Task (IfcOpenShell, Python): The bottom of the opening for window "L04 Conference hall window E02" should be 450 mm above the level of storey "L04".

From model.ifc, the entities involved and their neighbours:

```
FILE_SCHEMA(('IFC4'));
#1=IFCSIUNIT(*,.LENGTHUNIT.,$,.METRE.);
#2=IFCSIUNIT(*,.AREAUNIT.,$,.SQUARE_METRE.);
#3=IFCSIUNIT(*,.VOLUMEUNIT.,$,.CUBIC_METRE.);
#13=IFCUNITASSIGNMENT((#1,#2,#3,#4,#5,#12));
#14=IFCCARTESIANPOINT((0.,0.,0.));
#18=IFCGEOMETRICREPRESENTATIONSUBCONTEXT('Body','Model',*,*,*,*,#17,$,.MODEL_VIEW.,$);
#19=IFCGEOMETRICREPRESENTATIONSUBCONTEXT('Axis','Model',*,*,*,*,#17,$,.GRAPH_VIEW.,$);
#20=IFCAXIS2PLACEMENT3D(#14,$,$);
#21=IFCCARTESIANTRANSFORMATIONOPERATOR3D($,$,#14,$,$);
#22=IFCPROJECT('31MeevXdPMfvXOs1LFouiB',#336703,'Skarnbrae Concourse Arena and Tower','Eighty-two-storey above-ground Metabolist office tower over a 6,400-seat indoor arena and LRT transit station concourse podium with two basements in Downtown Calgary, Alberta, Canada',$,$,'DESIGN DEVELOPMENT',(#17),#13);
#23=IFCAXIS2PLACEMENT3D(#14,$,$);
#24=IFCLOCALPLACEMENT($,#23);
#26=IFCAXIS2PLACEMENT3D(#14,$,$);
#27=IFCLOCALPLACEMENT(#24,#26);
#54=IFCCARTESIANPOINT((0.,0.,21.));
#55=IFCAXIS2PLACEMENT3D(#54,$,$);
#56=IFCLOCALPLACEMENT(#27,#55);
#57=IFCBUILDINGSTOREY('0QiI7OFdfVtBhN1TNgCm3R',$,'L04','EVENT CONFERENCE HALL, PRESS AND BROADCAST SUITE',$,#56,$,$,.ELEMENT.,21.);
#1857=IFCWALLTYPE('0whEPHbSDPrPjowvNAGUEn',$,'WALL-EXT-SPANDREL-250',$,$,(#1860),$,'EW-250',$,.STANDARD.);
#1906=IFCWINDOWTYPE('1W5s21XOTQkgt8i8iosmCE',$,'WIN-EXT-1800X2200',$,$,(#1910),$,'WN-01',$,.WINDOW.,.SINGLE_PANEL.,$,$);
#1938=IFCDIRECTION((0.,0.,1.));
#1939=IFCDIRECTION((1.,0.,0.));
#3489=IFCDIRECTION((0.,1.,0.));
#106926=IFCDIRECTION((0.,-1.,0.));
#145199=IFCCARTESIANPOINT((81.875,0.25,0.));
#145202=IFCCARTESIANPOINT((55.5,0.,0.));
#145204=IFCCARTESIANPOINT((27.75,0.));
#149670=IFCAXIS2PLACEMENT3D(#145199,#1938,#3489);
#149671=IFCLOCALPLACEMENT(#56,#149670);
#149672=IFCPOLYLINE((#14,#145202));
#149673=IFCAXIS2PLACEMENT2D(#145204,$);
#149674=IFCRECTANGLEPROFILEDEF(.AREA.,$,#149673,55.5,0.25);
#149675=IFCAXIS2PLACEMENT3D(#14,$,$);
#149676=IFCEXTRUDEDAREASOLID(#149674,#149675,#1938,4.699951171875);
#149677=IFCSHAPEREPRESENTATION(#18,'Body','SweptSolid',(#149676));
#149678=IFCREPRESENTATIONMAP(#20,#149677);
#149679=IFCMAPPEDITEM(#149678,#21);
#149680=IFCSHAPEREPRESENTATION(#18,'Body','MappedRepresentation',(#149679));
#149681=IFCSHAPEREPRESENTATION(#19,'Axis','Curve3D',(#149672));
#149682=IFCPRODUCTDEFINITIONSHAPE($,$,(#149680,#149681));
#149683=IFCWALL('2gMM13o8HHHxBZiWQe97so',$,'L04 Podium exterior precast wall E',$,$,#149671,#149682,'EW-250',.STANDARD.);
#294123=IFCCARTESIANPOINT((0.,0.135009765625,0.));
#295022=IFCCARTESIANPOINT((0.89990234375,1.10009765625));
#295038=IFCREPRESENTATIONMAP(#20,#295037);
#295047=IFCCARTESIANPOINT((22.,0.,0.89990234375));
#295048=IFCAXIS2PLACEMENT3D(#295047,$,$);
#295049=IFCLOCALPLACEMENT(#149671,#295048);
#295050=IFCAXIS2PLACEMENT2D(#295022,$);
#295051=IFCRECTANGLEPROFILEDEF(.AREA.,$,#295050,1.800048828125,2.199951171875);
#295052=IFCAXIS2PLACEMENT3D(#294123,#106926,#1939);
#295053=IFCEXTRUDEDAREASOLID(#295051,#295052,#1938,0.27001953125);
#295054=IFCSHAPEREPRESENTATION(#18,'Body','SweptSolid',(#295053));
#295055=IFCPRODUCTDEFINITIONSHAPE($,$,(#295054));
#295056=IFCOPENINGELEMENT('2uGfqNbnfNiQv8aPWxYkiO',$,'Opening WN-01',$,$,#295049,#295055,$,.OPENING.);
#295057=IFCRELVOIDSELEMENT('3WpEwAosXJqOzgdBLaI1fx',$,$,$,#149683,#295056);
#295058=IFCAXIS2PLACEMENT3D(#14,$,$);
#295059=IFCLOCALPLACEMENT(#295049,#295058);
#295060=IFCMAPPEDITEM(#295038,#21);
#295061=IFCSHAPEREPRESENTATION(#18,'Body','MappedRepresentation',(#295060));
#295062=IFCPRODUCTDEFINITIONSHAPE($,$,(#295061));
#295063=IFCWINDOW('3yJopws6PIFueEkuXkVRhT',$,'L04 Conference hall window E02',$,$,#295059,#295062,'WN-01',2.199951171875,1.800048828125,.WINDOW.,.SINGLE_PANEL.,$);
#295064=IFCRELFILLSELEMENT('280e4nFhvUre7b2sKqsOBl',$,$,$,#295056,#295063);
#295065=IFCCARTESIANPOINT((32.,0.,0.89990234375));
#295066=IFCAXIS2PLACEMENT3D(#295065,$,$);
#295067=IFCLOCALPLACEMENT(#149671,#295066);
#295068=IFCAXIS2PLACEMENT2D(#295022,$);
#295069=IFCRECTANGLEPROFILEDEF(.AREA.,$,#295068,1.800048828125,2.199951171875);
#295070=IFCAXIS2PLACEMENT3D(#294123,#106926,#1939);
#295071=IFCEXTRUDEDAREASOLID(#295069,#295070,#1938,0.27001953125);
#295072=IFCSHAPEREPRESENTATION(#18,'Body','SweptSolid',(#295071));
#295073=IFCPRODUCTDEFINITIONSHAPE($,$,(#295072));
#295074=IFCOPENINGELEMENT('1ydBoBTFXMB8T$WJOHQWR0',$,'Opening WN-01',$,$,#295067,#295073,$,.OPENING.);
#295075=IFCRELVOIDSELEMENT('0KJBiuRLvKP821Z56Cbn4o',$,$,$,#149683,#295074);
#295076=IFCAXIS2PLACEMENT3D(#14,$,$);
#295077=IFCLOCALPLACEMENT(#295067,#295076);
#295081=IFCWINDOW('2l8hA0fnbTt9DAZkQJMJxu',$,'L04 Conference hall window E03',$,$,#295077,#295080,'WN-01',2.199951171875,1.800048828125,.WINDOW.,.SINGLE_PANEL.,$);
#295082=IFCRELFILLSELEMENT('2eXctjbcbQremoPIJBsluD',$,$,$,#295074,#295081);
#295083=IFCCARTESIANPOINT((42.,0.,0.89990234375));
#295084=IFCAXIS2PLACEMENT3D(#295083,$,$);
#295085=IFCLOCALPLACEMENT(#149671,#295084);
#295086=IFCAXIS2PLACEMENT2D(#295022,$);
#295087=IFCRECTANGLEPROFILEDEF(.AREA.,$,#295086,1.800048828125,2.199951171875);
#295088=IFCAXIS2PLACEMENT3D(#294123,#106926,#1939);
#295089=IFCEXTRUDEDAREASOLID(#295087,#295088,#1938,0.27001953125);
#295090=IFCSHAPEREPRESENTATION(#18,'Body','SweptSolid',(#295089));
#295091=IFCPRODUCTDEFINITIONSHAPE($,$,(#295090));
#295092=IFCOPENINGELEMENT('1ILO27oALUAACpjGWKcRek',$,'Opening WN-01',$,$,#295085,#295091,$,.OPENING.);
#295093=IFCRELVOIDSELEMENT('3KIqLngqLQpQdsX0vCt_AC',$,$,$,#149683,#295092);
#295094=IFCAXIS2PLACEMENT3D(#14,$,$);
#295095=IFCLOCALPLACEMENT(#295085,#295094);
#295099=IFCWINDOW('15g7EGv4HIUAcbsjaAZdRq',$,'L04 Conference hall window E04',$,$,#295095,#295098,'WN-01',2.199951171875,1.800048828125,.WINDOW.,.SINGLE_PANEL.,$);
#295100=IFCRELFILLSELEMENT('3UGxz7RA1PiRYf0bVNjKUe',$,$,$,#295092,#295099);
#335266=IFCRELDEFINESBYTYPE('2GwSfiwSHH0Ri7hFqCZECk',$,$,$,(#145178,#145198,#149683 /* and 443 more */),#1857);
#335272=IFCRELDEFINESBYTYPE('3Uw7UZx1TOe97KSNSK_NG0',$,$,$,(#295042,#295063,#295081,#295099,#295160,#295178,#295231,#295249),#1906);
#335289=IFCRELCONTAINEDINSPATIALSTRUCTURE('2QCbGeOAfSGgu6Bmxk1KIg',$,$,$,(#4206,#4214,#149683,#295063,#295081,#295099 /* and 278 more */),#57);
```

```python
import numpy as np
import ifcopenshell
import ifcopenshell.api.geometry
import ifcopenshell.geom
import ifcopenshell.util.element
import ifcopenshell.util.placement
import ifcopenshell.util.shape
import ifcopenshell.util.unit

model = ifcopenshell.open("model.ifc")
unit_scale = ifcopenshell.util.unit.calculate_unit_scale(model)

window = model.by_id(295063)
opening = window.FillsVoids[0].RelatingOpeningElement
storey = ifcopenshell.util.element.get_container(window, ifc_class="IfcBuildingStorey")
level = ifcopenshell.util.placement.get_local_placement(storey.ObjectPlacement)[2, 3]

# The opening's origin need not be at the sill, so measure its lowest point.
shape = ifcopenshell.geom.create_shape(ifcopenshell.geom.settings(), opening)
bottom = ifcopenshell.util.shape.get_shape_bottom_elevation(shape, shape.geometry) / unit_scale
dz = level + 0.45 / unit_scale - bottom

shift = np.array([0.0, 0.0, dz])
# The window is placed relative to its opening, so it follows when the opening moves.
matrix = ifcopenshell.util.placement.get_local_placement(opening.ObjectPlacement)
matrix[:3, 3] += shift
ifcopenshell.api.geometry.edit_object_placement(
    model, product=opening, matrix=matrix, is_si=False, should_transform_children=True
)

print(f"moved by {dz * unit_scale:+.3f} m")

model.write("model_edited.ifc")
```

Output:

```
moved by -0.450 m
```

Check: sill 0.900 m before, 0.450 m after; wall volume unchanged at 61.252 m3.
